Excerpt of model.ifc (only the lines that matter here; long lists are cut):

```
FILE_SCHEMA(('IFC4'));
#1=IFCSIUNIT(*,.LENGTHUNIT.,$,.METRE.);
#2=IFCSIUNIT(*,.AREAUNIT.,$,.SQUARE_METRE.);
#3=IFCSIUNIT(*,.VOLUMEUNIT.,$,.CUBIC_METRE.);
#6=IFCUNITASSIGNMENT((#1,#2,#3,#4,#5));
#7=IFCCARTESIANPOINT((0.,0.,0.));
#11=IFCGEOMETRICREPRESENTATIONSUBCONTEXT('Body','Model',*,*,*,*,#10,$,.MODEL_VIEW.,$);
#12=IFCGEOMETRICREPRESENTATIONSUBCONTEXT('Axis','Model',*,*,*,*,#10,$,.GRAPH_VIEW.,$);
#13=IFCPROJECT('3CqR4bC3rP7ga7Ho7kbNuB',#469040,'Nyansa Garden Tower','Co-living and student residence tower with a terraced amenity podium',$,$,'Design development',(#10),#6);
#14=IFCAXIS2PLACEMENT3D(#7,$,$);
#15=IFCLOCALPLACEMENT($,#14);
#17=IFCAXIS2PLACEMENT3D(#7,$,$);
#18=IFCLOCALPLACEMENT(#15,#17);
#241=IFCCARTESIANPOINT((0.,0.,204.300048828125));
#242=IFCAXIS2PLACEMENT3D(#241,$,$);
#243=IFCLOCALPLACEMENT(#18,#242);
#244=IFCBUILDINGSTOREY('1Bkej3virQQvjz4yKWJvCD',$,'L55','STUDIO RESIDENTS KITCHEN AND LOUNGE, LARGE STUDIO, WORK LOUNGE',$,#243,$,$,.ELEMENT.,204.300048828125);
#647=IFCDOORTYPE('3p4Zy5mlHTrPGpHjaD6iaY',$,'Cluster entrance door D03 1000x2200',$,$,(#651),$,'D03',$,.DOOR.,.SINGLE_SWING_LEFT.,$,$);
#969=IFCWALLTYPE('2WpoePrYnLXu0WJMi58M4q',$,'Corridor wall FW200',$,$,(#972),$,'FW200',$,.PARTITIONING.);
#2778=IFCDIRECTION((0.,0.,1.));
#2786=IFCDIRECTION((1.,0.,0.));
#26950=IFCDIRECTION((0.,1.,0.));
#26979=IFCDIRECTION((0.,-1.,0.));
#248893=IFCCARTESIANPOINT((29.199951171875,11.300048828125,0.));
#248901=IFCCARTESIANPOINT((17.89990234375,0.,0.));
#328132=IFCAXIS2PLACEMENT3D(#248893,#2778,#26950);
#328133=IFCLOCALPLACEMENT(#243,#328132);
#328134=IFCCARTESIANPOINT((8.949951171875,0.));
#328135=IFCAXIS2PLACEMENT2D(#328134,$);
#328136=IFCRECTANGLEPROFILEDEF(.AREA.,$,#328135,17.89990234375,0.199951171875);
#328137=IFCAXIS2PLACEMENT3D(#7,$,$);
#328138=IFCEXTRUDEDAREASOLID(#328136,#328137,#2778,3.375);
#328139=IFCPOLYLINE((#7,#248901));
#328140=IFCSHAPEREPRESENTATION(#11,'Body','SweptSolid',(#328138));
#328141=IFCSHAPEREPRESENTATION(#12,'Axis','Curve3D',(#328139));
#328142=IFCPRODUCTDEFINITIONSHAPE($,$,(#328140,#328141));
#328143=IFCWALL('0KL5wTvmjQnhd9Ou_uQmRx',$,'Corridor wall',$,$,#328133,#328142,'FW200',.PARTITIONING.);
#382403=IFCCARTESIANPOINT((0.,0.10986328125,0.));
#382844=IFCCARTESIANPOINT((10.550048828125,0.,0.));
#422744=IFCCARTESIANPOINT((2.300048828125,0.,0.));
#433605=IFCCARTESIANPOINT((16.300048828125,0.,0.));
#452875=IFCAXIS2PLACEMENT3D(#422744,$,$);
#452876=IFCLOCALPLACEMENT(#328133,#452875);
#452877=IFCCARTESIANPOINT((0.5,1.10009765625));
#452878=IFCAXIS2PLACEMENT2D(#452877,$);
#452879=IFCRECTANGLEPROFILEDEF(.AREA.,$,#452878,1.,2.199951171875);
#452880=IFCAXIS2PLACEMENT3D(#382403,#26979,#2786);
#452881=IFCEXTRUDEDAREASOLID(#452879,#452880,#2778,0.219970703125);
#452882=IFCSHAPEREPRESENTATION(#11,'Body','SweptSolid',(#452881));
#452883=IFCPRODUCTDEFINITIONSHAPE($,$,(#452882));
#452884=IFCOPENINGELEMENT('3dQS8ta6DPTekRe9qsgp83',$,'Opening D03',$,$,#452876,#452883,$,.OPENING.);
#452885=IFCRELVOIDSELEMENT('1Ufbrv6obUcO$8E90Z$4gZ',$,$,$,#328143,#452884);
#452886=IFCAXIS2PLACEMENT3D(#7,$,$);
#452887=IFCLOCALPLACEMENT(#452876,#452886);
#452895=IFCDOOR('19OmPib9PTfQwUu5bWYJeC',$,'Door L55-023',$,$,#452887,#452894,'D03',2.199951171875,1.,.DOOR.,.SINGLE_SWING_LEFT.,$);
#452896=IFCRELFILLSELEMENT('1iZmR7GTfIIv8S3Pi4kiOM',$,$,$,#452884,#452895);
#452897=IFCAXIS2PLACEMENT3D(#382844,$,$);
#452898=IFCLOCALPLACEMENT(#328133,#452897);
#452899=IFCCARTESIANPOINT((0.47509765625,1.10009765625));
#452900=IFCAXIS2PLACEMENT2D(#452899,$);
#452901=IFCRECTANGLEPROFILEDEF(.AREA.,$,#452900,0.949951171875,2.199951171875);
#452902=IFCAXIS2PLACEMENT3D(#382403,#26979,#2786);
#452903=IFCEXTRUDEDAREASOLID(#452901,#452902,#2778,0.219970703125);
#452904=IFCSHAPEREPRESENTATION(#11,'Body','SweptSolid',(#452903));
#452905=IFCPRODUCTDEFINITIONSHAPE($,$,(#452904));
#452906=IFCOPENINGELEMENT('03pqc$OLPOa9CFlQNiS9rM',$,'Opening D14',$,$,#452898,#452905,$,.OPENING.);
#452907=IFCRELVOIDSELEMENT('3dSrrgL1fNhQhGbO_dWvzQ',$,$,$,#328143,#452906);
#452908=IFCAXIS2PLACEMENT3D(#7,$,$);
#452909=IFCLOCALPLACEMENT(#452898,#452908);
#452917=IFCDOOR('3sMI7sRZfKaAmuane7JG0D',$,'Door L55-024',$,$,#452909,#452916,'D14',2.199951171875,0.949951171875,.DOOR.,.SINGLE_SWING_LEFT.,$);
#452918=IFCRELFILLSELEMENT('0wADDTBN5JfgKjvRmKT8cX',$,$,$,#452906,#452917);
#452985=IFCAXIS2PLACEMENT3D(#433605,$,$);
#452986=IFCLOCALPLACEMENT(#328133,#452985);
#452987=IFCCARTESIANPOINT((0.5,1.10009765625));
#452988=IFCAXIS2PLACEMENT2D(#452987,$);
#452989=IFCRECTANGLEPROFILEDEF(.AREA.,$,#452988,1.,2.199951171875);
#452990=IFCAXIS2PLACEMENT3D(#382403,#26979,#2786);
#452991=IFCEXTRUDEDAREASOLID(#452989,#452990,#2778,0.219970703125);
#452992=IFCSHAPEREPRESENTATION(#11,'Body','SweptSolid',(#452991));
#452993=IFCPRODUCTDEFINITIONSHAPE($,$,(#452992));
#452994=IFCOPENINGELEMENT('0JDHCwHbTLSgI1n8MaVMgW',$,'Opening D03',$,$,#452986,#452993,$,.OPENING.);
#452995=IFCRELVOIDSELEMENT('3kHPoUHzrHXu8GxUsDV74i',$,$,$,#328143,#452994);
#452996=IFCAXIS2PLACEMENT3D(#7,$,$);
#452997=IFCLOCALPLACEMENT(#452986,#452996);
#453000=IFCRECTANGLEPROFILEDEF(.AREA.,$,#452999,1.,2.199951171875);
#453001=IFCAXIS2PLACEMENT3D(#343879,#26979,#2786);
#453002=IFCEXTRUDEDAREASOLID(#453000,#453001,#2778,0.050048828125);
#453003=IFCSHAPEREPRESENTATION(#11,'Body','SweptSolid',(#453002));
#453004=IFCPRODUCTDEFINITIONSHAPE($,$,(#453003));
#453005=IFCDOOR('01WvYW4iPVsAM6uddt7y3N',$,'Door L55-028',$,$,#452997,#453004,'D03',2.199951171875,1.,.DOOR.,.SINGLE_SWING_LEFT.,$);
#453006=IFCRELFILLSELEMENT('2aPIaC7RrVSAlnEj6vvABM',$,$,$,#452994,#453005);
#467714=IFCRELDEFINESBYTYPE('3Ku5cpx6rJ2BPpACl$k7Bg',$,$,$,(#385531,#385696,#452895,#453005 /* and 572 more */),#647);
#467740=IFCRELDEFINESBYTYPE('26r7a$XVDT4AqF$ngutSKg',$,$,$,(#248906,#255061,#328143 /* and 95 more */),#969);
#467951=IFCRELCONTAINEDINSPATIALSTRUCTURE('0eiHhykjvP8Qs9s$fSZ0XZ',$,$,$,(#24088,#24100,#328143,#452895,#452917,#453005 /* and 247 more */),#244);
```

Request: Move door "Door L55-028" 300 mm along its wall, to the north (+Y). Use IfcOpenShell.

```python
import ifcopenshell
import ifcopenshell.api.geometry
import ifcopenshell.util.placement

model = ifcopenshell.open("model.ifc")

door = model.by_id(453005)
opening = door.FillsVoids[0].RelatingOpeningElement
wall = opening.VoidsElements[0].RelatingBuildingElement

wall_matrix = ifcopenshell.util.placement.get_local_placement(wall.ObjectPlacement)
shift = wall_matrix[:3, 0] * 0.3
before = ifcopenshell.util.placement.get_local_placement(door.ObjectPlacement)[:3, 3].copy()

# The door is placed relative to its opening, so it follows when the opening moves.
matrix = ifcopenshell.util.placement.get_local_placement(opening.ObjectPlacement)
matrix[:3, 3] += shift
ifcopenshell.api.geometry.edit_object_placement(
    model, product=opening, matrix=matrix, is_si=False, should_transform_children=True
)

after = ifcopenshell.util.placement.get_local_placement(door.ObjectPlacement)[:3, 3]
print("door moved by", (after - before).round(3) + 0.0)

model.write("model_updated.ifc")
```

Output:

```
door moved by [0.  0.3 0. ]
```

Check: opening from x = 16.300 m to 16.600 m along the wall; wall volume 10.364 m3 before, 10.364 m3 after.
